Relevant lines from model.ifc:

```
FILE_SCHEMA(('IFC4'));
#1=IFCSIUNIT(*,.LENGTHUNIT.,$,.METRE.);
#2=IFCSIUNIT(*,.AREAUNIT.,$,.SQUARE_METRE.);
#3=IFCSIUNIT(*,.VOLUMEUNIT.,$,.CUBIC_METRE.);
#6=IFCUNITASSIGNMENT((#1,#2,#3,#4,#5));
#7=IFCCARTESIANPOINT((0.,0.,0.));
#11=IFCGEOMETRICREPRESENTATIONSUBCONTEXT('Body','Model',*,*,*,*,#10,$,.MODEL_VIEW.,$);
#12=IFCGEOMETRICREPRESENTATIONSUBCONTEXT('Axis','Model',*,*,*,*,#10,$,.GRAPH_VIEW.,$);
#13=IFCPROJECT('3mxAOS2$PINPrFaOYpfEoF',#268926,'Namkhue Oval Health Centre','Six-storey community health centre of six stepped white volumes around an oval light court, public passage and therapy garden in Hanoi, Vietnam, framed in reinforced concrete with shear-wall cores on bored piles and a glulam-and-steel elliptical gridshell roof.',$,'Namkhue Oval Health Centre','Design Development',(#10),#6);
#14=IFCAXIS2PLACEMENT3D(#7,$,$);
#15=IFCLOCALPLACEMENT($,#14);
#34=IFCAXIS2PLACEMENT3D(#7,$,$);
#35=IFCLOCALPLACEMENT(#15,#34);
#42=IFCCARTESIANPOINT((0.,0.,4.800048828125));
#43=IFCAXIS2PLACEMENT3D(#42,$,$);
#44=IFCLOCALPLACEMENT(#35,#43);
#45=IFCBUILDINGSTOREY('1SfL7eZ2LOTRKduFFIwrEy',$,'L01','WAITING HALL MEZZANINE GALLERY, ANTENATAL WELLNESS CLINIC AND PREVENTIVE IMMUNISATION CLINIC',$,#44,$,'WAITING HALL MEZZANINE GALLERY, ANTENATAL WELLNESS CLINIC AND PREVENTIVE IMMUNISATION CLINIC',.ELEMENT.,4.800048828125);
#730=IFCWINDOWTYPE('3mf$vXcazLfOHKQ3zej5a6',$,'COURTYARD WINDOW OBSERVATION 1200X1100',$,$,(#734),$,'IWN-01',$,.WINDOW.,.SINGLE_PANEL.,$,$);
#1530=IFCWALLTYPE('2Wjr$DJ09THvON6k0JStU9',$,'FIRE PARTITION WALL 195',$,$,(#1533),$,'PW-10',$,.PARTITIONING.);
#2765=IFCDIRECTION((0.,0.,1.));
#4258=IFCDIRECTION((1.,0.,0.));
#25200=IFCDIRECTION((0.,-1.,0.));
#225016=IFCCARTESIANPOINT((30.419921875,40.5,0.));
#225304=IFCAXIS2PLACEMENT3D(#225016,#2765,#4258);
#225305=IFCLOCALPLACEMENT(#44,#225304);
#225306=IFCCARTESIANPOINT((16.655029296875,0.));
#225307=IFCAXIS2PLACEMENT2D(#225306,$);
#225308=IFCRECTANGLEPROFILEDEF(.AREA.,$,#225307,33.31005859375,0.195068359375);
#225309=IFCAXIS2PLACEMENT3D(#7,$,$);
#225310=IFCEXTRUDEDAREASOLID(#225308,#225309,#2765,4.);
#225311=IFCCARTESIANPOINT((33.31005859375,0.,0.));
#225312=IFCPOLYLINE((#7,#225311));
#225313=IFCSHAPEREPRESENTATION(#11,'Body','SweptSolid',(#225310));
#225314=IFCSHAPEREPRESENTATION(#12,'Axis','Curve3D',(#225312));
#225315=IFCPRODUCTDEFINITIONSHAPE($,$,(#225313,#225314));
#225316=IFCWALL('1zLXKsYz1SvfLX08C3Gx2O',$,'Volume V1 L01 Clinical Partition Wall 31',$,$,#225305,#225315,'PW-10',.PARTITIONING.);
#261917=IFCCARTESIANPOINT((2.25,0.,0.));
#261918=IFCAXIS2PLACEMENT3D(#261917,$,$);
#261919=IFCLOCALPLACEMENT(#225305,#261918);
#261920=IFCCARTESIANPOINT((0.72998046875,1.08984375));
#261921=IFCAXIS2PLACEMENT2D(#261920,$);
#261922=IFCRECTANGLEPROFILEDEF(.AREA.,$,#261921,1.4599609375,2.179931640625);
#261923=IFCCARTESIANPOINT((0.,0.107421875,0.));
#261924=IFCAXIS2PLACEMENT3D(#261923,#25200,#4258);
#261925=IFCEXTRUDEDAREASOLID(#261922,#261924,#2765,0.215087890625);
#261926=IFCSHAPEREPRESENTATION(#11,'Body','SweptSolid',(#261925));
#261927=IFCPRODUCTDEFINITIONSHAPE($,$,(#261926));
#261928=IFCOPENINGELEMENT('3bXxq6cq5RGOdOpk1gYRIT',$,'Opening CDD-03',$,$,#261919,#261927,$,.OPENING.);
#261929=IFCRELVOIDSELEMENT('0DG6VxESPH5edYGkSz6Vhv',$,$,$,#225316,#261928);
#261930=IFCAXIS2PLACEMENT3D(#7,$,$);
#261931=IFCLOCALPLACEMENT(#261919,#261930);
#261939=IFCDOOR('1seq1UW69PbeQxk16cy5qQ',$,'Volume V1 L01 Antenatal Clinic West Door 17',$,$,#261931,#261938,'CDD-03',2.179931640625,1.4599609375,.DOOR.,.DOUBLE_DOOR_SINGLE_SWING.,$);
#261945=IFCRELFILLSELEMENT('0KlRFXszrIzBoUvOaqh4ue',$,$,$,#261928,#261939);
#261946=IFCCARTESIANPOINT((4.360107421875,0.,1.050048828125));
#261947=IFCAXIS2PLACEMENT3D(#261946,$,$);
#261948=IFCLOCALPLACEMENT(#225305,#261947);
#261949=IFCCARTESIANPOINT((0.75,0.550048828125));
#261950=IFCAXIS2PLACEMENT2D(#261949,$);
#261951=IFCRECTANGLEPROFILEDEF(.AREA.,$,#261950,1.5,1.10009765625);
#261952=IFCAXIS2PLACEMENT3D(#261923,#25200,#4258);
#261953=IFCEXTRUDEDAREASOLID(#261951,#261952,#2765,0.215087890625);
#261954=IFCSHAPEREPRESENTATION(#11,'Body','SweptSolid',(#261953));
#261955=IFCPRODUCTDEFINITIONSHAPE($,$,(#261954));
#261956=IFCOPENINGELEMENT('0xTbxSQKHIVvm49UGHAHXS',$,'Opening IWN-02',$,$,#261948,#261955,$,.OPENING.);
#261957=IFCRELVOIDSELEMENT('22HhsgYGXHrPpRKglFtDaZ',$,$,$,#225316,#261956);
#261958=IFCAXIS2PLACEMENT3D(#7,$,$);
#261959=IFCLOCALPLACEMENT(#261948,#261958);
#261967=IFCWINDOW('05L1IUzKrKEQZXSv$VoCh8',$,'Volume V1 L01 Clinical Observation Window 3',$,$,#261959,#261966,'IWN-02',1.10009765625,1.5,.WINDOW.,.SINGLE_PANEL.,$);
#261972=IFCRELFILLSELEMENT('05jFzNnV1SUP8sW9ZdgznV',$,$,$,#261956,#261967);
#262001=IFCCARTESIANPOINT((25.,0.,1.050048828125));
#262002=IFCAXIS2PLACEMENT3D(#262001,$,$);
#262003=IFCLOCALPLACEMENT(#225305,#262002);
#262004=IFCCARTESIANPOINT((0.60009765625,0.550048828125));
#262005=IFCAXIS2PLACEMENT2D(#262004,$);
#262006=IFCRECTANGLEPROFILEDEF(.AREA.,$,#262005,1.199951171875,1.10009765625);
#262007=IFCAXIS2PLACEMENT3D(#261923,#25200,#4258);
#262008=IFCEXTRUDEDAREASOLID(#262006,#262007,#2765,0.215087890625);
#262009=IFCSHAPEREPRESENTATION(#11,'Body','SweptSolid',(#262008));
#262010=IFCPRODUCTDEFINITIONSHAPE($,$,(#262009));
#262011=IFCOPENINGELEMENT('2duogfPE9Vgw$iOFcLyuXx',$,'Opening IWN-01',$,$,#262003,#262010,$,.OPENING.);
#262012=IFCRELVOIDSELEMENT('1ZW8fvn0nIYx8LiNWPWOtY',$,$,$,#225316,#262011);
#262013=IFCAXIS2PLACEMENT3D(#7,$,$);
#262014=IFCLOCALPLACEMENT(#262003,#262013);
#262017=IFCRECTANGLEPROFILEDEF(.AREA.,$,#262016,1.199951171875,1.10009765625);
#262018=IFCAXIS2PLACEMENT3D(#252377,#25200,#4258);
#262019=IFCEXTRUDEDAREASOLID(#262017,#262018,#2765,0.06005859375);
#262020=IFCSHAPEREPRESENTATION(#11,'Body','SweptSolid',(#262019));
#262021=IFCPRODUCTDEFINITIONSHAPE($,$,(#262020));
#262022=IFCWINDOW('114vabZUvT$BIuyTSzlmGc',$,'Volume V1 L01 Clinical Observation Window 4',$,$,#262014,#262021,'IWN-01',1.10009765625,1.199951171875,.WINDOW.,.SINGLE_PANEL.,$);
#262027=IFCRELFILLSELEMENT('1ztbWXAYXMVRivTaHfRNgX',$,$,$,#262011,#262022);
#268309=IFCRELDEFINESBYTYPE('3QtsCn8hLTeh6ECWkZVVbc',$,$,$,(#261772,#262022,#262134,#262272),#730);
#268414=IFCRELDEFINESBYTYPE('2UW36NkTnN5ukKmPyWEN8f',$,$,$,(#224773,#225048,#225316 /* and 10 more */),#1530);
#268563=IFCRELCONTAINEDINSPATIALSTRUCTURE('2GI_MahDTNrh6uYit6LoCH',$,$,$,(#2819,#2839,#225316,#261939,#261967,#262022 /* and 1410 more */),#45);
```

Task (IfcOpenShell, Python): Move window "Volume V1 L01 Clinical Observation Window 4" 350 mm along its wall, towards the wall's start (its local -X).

```python
import ifcopenshell
import ifcopenshell.api.geometry
import ifcopenshell.util.placement
import ifcopenshell.util.unit

model = ifcopenshell.open("model.ifc")
unit_scale = ifcopenshell.util.unit.calculate_unit_scale(model)

window = model.by_guid("114vabZUvT$BIuyTSzlmGc")
opening = window.FillsVoids[0].RelatingOpeningElement
wall = opening.VoidsElements[0].RelatingBuildingElement

wall_matrix = ifcopenshell.util.placement.get_local_placement(wall.ObjectPlacement)
shift = wall_matrix[:3, 0] * -0.35 / unit_scale
before = ifcopenshell.util.placement.get_local_placement(window.ObjectPlacement)[:3, 3].copy()

# The window is placed relative to its opening, so it follows when the opening moves.
matrix = ifcopenshell.util.placement.get_local_placement(opening.ObjectPlacement)
matrix[:3, 3] += shift
ifcopenshell.api.geometry.edit_object_placement(
    model, product=opening, matrix=matrix, is_si=False, should_transform_children=True
)

after = ifcopenshell.util.placement.get_local_placement(window.ObjectPlacement)[:3, 3]
print("window moved by", (after - before).round(3) + 0.0)

model.write("model-out.ifc")
```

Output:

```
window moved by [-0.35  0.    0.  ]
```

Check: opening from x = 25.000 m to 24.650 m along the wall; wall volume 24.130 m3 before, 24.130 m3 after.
